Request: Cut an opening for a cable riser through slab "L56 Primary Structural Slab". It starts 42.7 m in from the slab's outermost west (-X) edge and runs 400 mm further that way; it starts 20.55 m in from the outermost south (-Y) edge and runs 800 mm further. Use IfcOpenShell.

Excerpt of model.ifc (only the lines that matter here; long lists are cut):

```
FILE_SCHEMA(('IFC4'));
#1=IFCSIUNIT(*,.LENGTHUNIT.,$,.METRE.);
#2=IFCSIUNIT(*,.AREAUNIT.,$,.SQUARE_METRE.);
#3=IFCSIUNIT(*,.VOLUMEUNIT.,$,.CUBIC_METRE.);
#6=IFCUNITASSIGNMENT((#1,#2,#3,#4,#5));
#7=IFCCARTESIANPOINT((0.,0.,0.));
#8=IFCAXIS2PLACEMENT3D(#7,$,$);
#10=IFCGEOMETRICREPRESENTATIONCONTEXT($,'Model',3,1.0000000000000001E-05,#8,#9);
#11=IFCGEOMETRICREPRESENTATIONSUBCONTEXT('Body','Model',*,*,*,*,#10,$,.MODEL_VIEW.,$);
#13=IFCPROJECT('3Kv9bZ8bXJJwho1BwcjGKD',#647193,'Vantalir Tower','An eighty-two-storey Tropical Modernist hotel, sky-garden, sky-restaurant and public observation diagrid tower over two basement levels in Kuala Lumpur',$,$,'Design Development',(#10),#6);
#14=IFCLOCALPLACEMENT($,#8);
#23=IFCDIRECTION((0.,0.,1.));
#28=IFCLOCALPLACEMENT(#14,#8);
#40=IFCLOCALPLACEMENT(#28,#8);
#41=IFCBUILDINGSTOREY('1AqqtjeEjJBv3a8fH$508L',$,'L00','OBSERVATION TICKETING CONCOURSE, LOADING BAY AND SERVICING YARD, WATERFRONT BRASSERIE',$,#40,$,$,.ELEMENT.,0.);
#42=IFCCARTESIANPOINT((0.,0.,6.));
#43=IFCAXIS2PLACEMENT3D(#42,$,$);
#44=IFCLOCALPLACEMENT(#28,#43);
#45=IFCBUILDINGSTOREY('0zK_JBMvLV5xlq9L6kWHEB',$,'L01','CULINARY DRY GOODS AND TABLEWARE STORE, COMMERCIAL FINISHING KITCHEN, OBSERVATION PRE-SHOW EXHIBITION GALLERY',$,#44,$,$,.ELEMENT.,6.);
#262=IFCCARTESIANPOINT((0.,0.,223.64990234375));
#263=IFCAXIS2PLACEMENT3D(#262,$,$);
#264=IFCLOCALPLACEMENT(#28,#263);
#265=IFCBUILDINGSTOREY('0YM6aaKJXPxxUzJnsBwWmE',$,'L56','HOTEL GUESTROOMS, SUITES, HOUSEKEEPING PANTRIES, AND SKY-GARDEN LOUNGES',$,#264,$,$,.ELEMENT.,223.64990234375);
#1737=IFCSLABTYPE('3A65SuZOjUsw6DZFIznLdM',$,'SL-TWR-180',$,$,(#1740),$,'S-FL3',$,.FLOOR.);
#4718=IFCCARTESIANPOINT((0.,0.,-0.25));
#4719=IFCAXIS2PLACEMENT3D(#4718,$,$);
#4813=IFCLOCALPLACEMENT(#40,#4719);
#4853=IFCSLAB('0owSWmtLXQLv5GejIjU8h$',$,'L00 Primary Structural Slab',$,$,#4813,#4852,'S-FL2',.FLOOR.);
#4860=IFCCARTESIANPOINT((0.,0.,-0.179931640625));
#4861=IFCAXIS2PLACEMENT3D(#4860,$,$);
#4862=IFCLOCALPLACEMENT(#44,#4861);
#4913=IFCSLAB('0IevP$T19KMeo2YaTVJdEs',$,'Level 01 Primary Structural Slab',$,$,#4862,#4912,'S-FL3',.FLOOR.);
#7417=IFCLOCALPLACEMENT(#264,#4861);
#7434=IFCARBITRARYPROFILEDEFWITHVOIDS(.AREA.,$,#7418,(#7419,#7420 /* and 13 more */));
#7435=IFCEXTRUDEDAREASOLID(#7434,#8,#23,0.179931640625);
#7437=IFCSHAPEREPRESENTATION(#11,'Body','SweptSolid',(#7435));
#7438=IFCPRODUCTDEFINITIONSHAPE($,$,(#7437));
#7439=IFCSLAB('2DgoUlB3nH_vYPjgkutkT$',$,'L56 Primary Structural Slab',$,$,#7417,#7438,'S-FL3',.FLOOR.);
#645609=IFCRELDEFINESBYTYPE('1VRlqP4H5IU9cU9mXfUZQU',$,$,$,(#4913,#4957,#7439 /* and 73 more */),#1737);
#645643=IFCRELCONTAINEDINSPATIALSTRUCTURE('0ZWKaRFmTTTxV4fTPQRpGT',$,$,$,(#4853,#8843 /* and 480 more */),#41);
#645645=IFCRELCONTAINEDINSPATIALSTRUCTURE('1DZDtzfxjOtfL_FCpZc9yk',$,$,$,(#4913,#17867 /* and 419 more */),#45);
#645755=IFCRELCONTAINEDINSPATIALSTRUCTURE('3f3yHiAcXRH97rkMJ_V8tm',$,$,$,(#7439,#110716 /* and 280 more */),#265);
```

```python
import numpy as np
import ifcopenshell
import ifcopenshell.api.feature
import ifcopenshell.api.geometry
import ifcopenshell.api.root
import ifcopenshell.geom
import ifcopenshell.util.placement
import ifcopenshell.util.representation
import ifcopenshell.util.shape
import ifcopenshell.util.unit

model = ifcopenshell.open("model.ifc")
unit_scale = ifcopenshell.util.unit.calculate_unit_scale(model)
settings = ifcopenshell.geom.settings()


def volume(element):
    """Net volume in cubic metres, openings subtracted."""
    shape = ifcopenshell.geom.create_shape(settings, element)
    return ifcopenshell.util.shape.get_volume(shape.geometry)


slab = model.by_guid("2DgoUlB3nH_vYPjgkutkT$")
before = volume(slab)

# Extent in the slab's own axes, in metres. The edges named are its -X and -Y sides.
slab_shape = ifcopenshell.geom.create_shape(settings, slab)
vertices = ifcopenshell.util.shape.get_vertices(slab_shape.geometry)
x_min, y_min, bottom = vertices.min(axis=0)
top = vertices[:, 2].max()

opening = ifcopenshell.api.root.create_entity(model, ifc_class="IfcOpeningElement", name="Cable riser opening", predefined_type="OPENING")
context = ifcopenshell.util.representation.get_context(model, "Model", "Body", "MODEL_VIEW")
width, depth = 0.4, 0.8
outline = [(0.0, 0.0), (width, 0.0), (width, depth), (0.0, depth), (0.0, 0.0)]
# Overshoot both faces by 50 mm so the cut is clean.
shape = ifcopenshell.api.geometry.add_slab_representation(
    model, context=context, depth=top - bottom + 0.1, polyline=outline
)
ifcopenshell.api.geometry.assign_representation(model, product=opening, representation=shape)

matrix = ifcopenshell.util.placement.get_local_placement(slab.ObjectPlacement)
matrix[:, 3] = matrix @ np.append(np.array([x_min + 42.7, y_min + 20.55, bottom - 0.05]) / unit_scale, 1.0)
ifcopenshell.api.geometry.edit_object_placement(model, product=opening, matrix=matrix, is_si=False)
ifcopenshell.api.feature.add_feature(model, feature=opening, element=slab)

after = volume(slab)

print(f"slab volume {before:.3f} -> {after:.3f} m3")

model.write("model_updated.ifc")
```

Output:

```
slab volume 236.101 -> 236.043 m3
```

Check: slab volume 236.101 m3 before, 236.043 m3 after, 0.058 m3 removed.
